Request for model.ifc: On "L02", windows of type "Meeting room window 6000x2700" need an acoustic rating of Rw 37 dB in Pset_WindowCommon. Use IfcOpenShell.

First a look at what the model holds.

```python
import ifcopenshell
import ifcopenshell.util.element

model = ifcopenshell.open("model.ifc")
print(model.schema)
storey = next(s for s in model.by_type("IfcBuildingStorey") if s.Name == "L02")
windows = [e for e in ifcopenshell.util.element.get_decomposition(storey) if e.is_a("IfcWindow")]
seen = {}
for e in windows:
    element_type = ifcopenshell.util.element.get_type(e)
    key = (element_type.Name if element_type != e and element_type else None, ifcopenshell.util.element.get_pset(e, "Pset_WindowCommon", "AcousticRating"))
    seen[key] = seen.get(key, 0) + 1
for (name, value), count in sorted(seen.items(), key=str):
    print(count, "x", name, "|", value)
```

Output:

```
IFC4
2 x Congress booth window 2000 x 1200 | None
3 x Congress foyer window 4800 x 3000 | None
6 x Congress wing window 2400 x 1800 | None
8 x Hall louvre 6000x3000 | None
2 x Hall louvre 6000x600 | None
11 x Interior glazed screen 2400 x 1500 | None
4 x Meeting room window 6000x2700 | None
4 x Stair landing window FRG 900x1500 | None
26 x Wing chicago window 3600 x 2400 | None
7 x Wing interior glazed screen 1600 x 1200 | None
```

```python
import ifcopenshell
import ifcopenshell.api.pset
import ifcopenshell.util.element

model = ifcopenshell.open("model.ifc")

storey = next(s for s in model.by_type("IfcBuildingStorey") if s.Name == "L02")
windows = [e for e in ifcopenshell.util.element.get_decomposition(storey) if e.is_a("IfcWindow")]

count = 0
for e in windows:
    element_type = ifcopenshell.util.element.get_type(e)
    if element_type in (None, e) or element_type.Name != "Meeting room window 6000x2700":
        continue
    # add_pset returns the element's existing set when there is one.
    pset = ifcopenshell.api.pset.add_pset(model, product=e, name="Pset_WindowCommon")
    ifcopenshell.api.pset.edit_pset(model, pset=pset, properties={"AcousticRating": "Rw 37 dB"})
    count += 1

print(count, "windows updated")

model.write("model_edited.ifc")
```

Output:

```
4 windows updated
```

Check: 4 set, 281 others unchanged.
